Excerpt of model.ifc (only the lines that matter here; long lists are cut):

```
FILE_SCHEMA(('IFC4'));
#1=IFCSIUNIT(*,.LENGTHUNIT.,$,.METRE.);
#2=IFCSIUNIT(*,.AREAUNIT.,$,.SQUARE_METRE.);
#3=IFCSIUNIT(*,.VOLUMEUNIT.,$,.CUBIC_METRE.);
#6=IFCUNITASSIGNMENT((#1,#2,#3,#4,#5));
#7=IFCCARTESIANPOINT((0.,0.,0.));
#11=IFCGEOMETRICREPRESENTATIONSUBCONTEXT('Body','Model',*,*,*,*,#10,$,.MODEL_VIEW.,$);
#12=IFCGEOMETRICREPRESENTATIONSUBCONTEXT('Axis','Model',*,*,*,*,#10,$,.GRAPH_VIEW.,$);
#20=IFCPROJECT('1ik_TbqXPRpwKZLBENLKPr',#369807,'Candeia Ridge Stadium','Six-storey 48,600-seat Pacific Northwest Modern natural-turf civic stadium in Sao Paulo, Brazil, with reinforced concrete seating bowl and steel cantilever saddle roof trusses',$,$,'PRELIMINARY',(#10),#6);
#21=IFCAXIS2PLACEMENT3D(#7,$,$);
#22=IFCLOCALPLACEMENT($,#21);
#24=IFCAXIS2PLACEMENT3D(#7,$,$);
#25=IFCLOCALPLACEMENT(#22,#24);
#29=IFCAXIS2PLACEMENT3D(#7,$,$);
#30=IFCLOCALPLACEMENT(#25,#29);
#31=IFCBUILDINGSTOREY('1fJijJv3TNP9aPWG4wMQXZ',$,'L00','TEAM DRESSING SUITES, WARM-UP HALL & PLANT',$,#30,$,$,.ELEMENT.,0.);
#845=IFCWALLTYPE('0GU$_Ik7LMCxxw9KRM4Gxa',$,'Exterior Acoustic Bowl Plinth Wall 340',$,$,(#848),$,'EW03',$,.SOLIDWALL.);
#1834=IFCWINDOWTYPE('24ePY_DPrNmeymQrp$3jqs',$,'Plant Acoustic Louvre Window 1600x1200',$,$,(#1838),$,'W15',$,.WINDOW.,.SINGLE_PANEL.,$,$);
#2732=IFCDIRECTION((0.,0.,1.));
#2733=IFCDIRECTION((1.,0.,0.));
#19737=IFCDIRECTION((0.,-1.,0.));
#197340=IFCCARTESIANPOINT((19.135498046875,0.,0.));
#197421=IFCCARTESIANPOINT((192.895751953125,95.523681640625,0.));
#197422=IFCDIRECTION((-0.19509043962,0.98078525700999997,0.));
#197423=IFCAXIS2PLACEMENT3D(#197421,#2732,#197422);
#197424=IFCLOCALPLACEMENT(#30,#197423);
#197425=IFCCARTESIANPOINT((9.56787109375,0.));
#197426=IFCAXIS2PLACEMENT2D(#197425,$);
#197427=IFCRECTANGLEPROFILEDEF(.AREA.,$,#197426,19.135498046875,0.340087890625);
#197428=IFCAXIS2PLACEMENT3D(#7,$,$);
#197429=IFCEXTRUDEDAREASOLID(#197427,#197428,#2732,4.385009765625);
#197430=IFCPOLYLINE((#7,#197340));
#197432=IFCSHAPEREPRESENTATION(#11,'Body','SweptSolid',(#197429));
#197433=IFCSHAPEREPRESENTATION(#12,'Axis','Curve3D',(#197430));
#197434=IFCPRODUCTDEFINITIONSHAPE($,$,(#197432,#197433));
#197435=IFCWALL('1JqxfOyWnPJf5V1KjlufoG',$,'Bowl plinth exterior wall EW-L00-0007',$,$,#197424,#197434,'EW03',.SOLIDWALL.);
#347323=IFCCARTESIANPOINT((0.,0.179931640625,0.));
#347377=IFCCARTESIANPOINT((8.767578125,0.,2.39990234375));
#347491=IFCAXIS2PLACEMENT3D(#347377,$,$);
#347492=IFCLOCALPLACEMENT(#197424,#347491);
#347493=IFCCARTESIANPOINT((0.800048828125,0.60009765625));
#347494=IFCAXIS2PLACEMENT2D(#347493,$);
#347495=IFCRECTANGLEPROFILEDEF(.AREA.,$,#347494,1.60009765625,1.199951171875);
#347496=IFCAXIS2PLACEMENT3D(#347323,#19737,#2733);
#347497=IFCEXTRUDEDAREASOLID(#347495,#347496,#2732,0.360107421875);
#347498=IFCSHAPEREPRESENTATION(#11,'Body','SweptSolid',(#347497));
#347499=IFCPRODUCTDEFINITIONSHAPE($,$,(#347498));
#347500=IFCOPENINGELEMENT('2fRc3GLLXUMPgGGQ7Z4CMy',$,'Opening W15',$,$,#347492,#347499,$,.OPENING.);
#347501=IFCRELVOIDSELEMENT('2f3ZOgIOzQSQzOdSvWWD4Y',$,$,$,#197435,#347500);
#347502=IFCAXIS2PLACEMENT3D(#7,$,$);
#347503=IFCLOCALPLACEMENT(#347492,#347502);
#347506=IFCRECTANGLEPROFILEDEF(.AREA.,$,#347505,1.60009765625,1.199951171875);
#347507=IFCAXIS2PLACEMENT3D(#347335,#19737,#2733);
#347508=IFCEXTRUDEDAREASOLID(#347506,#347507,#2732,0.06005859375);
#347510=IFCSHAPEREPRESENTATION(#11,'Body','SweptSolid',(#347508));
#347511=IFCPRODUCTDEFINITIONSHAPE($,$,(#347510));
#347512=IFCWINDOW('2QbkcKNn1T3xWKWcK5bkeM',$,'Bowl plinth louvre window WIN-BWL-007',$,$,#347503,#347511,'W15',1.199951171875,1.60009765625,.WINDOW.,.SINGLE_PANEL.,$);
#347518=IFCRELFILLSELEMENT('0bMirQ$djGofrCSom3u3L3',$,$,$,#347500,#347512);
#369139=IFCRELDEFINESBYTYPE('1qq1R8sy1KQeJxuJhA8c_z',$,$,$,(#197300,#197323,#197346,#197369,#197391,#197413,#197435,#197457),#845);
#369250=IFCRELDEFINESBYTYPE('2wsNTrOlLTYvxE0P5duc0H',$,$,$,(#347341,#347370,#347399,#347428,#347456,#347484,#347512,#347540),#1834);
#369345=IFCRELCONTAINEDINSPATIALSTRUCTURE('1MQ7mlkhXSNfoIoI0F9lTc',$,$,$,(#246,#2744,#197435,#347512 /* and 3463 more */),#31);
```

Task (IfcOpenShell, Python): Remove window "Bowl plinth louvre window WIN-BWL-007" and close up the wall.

```python
import ifcopenshell
import ifcopenshell.api.feature
import ifcopenshell.api.root
import ifcopenshell.geom
import ifcopenshell.util.shape

model = ifcopenshell.open("model.ifc")
settings = ifcopenshell.geom.settings()


def volume(element):
    """Net volume in cubic metres, openings subtracted."""
    shape = ifcopenshell.geom.create_shape(settings, element)
    return ifcopenshell.util.shape.get_volume(shape.geometry)


window = model.by_guid("2QbkcKNn1T3xWKWcK5bkeM")
opening = window.FillsVoids[0].RelatingOpeningElement
wall = opening.VoidsElements[0].RelatingBuildingElement
before = volume(wall)

ifcopenshell.api.root.remove_product(model, product=window)
ifcopenshell.api.feature.remove_feature(model, feature=opening)

after = volume(wall)

print(f"wall volume {before:.3f} -> {after:.3f} m3")

model.write("model_edited.ifc")
```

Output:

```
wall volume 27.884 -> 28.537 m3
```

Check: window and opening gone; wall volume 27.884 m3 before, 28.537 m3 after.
